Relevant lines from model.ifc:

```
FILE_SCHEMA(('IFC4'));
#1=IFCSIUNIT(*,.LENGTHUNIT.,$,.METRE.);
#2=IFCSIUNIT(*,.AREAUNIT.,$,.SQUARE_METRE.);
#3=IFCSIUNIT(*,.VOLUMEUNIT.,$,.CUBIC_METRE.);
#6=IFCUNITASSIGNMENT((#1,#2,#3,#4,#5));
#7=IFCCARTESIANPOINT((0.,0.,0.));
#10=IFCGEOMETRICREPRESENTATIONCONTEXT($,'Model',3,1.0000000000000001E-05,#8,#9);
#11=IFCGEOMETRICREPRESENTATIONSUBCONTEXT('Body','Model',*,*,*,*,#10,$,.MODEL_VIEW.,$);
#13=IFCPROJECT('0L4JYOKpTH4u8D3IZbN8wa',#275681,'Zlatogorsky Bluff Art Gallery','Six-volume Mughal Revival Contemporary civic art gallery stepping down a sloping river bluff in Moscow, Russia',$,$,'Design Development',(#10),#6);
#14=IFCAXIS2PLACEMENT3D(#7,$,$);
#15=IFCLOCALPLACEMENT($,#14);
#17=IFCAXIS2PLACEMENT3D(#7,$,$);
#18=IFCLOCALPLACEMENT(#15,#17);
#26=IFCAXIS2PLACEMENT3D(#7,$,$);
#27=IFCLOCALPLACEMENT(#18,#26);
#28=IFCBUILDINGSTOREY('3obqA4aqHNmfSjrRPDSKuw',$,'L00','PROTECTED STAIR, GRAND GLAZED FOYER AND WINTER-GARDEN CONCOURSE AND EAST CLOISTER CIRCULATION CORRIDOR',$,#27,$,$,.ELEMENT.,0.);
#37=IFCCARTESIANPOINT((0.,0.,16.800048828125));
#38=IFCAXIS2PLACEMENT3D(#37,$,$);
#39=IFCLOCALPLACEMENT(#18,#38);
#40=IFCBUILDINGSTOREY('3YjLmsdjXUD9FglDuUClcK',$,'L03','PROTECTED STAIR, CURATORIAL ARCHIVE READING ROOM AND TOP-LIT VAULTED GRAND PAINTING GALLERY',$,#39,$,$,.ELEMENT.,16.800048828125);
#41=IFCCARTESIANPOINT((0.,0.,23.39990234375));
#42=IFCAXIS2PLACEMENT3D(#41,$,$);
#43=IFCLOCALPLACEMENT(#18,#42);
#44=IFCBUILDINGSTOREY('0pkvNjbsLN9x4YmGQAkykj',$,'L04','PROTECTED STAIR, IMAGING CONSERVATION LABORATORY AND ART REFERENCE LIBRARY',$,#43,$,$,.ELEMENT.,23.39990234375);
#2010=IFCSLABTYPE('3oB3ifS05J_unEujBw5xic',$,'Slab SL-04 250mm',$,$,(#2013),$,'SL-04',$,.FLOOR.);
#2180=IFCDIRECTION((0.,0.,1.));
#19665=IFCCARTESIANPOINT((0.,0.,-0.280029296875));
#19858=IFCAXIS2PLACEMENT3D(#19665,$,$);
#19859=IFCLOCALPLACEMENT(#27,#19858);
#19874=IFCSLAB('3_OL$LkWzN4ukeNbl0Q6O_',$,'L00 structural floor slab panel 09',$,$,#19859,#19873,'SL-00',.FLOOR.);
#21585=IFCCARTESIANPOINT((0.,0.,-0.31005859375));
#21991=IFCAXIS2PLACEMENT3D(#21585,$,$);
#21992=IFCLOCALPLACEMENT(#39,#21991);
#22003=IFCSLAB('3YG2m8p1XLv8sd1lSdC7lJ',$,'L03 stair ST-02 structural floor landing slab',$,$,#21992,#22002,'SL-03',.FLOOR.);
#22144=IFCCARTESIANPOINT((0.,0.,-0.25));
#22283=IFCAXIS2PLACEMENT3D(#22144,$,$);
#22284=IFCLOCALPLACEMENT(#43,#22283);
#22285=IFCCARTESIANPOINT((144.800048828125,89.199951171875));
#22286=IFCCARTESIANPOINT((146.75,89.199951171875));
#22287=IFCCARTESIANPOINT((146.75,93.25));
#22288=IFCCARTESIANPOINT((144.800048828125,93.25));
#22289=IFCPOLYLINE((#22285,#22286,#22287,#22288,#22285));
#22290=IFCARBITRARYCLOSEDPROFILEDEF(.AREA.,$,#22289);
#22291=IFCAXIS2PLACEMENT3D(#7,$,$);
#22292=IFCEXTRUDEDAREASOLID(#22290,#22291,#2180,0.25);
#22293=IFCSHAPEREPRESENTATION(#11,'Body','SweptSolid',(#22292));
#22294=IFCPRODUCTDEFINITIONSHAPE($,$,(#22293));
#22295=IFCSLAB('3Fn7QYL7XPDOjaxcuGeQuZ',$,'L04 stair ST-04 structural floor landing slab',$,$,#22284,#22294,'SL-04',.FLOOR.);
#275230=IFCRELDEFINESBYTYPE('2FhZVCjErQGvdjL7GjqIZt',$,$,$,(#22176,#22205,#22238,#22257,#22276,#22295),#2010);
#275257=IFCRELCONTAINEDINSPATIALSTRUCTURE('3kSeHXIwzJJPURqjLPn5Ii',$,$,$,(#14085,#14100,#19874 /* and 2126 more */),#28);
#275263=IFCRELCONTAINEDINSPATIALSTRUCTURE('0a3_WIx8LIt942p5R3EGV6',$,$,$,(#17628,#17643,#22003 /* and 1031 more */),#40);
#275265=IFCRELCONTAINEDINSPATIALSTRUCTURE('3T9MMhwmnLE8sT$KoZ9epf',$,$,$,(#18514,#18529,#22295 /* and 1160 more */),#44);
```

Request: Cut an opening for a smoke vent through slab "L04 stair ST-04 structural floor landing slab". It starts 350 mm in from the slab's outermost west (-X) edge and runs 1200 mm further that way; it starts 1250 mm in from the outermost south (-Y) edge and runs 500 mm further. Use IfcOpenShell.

```python
import numpy as np
import ifcopenshell
import ifcopenshell.api.feature
import ifcopenshell.api.geometry
import ifcopenshell.api.root
import ifcopenshell.geom
import ifcopenshell.util.placement
import ifcopenshell.util.representation
import ifcopenshell.util.shape
import ifcopenshell.util.unit

model = ifcopenshell.open("model.ifc")
unit_scale = ifcopenshell.util.unit.calculate_unit_scale(model)
settings = ifcopenshell.geom.settings()


def volume(element):
    """Net volume in cubic metres, openings subtracted."""
    shape = ifcopenshell.geom.create_shape(settings, element)
    return ifcopenshell.util.shape.get_volume(shape.geometry)


slab = model.by_guid("3Fn7QYL7XPDOjaxcuGeQuZ")
before = volume(slab)

# Extent in the slab's own axes, in metres. The edges named are its -X and -Y sides.
slab_shape = ifcopenshell.geom.create_shape(settings, slab)
vertices = ifcopenshell.util.shape.get_vertices(slab_shape.geometry)
x_min, y_min, bottom = vertices.min(axis=0)
top = vertices[:, 2].max()

opening = ifcopenshell.api.root.create_entity(model, ifc_class="IfcOpeningElement", name="Smoke vent opening", predefined_type="OPENING")
context = ifcopenshell.util.representation.get_context(model, "Model", "Body", "MODEL_VIEW")
width, depth = 1.2, 0.5
outline = [(0.0, 0.0), (width, 0.0), (width, depth), (0.0, depth), (0.0, 0.0)]
# Overshoot both faces by 50 mm so the cut is clean.
shape = ifcopenshell.api.geometry.add_slab_representation(
    model, context=context, depth=top - bottom + 0.1, polyline=outline
)
ifcopenshell.api.geometry.assign_representation(model, product=opening, representation=shape)

matrix = ifcopenshell.util.placement.get_local_placement(slab.ObjectPlacement)
matrix[:, 3] = matrix @ np.append(np.array([x_min + 0.35, y_min + 1.25, bottom - 0.05]) / unit_scale, 1.0)
ifcopenshell.api.geometry.edit_object_placement(model, product=opening, matrix=matrix, is_si=False)
ifcopenshell.api.feature.add_feature(model, feature=opening, element=slab)

after = volume(slab)

print(f"slab volume {before:.3f} -> {after:.3f} m3")

model.write("model-out.ifc")
```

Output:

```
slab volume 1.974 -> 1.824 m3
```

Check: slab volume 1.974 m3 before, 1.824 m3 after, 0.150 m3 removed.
